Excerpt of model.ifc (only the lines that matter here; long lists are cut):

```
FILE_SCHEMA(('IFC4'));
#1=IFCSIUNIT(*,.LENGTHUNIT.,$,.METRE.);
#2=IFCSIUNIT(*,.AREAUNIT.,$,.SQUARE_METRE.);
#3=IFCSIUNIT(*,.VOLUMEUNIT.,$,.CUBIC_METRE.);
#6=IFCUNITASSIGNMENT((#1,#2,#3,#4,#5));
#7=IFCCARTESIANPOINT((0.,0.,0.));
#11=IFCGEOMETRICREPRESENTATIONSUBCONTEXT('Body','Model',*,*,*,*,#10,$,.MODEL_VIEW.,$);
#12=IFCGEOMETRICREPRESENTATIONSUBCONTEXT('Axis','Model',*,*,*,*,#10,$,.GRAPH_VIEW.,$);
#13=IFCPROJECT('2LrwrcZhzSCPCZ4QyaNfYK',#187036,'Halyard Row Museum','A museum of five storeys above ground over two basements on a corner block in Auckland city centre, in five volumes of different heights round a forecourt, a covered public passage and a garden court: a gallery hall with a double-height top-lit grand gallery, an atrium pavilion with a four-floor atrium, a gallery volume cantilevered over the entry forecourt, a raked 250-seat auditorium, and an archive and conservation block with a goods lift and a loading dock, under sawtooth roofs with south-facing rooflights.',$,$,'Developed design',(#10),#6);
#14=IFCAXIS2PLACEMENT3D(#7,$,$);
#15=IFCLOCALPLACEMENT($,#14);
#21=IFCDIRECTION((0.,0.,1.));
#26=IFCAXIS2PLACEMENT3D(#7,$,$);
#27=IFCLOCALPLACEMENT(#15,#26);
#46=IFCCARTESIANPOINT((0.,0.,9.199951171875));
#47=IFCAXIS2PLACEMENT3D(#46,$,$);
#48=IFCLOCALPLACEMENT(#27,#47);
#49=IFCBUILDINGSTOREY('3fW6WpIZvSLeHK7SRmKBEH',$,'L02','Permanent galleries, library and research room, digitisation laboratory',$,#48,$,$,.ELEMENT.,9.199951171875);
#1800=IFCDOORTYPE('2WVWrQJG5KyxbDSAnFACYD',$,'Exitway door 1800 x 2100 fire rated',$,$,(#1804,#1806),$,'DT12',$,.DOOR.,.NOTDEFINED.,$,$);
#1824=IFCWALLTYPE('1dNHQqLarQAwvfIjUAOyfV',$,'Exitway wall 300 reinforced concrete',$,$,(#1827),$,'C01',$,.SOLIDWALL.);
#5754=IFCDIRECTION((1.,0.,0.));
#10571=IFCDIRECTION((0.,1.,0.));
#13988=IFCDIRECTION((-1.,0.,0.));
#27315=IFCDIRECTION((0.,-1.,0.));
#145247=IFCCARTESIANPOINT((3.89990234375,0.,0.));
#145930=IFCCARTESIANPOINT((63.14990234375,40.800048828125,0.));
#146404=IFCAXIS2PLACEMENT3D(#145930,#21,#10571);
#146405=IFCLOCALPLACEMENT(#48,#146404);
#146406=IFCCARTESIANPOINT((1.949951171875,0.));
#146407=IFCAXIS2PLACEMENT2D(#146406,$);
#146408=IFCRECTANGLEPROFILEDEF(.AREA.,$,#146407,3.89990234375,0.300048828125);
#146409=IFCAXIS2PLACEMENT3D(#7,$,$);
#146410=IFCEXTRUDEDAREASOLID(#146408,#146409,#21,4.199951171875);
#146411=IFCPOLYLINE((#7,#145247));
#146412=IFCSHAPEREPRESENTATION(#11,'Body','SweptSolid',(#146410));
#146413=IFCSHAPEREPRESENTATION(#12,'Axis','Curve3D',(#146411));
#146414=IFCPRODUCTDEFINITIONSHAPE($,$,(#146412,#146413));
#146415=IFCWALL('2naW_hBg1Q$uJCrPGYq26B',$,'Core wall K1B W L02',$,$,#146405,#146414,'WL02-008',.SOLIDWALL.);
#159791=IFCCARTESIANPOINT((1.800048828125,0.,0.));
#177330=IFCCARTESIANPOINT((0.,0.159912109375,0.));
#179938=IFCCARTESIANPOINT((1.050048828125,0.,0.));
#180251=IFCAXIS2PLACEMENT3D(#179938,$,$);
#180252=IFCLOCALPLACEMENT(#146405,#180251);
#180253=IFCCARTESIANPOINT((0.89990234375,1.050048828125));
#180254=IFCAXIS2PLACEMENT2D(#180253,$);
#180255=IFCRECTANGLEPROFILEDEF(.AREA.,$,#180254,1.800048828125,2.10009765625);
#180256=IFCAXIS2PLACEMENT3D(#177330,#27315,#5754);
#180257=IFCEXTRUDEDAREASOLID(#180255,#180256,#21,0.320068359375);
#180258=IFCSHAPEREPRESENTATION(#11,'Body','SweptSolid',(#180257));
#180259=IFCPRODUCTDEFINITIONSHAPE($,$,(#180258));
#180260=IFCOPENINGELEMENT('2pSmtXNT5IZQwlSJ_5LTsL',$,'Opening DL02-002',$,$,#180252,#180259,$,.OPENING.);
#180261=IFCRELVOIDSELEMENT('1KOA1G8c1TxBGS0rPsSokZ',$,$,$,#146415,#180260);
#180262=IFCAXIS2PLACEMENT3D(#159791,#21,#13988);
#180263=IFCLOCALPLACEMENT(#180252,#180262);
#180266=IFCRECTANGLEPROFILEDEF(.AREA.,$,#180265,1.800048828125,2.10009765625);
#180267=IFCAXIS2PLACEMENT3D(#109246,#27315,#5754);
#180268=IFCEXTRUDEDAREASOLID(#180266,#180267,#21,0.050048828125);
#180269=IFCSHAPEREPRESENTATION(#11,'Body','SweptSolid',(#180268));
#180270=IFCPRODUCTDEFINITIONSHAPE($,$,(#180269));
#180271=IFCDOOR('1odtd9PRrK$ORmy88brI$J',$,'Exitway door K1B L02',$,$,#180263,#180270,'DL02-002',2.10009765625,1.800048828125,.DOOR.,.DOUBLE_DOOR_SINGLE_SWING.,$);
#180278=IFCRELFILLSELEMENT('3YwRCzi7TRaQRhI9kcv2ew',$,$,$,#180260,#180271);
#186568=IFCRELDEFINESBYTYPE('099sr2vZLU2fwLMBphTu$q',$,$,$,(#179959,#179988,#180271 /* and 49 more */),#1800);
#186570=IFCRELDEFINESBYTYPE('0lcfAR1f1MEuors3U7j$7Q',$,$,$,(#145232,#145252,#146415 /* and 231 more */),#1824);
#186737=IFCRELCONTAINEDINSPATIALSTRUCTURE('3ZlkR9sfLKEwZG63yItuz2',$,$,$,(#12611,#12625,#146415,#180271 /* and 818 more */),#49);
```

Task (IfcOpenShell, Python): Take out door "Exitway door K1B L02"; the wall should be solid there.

```python
import ifcopenshell
import ifcopenshell.api.feature
import ifcopenshell.api.root
import ifcopenshell.geom
import ifcopenshell.util.shape

model = ifcopenshell.open("model.ifc")
settings = ifcopenshell.geom.settings()


def volume(element):
    """Net volume in cubic metres, openings subtracted."""
    shape = ifcopenshell.geom.create_shape(settings, element)
    return ifcopenshell.util.shape.get_volume(shape.geometry)


door = model.by_guid("1odtd9PRrK$ORmy88brI$J")
opening = door.FillsVoids[0].RelatingOpeningElement
wall = opening.VoidsElements[0].RelatingBuildingElement
before = volume(wall)

ifcopenshell.api.root.remove_product(model, product=door)
ifcopenshell.api.feature.remove_feature(model, feature=opening)

after = volume(wall)

print(f"wall volume {before:.3f} -> {after:.3f} m3")

model.write("model_updated.ifc")
```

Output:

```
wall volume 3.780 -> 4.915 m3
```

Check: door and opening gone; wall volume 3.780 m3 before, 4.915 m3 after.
